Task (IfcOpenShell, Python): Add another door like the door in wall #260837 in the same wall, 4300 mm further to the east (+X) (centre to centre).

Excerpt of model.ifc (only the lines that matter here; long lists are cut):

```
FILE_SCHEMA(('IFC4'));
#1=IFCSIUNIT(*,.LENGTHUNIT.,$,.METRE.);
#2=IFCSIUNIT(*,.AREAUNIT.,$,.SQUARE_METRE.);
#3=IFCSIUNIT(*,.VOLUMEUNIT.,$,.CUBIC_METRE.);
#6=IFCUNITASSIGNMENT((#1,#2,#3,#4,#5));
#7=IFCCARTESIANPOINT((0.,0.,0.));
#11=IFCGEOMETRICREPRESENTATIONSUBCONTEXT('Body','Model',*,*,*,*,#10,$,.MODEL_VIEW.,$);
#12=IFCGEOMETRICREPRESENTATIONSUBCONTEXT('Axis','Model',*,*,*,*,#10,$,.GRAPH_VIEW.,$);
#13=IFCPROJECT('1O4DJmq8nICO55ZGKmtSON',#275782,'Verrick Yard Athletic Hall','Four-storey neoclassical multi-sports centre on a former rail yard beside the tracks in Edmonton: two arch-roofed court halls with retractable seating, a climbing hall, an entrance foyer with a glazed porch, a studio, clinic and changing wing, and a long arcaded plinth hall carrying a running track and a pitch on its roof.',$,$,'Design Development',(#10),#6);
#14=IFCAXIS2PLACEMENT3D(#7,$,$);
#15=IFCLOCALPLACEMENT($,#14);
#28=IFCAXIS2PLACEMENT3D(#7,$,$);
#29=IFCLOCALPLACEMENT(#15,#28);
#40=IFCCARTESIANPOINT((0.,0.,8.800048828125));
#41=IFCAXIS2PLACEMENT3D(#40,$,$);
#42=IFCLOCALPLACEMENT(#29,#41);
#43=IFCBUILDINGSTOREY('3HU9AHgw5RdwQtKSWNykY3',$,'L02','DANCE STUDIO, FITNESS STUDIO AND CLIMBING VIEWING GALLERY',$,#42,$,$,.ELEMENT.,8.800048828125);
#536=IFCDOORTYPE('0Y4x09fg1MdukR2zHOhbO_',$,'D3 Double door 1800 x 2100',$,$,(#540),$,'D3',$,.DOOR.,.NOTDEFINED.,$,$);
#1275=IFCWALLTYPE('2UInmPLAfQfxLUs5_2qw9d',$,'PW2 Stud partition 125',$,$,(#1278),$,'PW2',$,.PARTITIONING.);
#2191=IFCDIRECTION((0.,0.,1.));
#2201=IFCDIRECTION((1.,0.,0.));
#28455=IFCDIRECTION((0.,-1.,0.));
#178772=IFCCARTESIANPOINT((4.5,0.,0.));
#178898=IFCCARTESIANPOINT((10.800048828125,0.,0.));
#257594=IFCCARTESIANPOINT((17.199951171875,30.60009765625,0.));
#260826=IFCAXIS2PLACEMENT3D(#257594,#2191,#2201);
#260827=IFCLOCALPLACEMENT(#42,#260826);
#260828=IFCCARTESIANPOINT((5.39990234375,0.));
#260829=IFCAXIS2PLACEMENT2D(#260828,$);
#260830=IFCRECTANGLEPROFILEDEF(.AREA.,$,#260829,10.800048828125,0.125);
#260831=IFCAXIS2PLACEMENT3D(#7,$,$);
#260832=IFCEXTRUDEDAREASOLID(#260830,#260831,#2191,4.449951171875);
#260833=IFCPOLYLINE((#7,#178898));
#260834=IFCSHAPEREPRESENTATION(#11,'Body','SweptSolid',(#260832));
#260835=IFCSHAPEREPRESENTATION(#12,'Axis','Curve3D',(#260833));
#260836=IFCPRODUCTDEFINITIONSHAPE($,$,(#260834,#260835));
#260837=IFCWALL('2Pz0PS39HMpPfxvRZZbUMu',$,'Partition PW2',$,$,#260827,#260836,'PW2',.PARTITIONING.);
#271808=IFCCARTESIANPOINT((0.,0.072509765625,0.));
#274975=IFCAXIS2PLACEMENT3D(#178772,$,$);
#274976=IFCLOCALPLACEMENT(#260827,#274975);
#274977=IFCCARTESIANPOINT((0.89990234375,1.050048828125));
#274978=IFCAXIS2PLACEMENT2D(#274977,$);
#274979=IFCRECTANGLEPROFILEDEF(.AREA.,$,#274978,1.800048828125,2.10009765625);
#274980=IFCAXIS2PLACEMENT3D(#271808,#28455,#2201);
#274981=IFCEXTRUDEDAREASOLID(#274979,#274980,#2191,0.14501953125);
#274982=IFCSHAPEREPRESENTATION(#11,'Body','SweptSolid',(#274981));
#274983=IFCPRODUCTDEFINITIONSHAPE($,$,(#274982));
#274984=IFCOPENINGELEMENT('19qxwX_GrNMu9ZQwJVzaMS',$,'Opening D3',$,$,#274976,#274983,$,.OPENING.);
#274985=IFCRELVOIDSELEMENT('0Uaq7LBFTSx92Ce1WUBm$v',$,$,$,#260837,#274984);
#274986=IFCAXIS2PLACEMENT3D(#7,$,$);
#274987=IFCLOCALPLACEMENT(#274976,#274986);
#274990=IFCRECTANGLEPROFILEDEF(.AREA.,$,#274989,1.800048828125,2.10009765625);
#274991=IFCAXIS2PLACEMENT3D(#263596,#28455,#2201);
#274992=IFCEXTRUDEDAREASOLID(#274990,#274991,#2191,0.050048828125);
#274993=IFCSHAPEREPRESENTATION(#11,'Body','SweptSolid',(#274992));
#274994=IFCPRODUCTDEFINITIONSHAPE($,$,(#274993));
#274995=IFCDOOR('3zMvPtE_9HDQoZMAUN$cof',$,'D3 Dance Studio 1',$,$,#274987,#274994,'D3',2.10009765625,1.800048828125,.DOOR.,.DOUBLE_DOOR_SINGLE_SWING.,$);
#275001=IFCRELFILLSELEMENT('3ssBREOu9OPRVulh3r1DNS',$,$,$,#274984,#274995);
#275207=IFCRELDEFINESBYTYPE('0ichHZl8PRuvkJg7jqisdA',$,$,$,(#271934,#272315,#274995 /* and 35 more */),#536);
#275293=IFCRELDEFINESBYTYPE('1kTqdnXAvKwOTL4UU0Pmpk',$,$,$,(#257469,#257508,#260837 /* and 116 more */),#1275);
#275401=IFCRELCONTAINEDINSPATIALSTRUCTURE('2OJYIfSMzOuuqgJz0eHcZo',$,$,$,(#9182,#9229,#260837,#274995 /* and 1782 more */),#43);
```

```python
import ifcopenshell
import ifcopenshell.api.feature
import ifcopenshell.api.geometry
import ifcopenshell.api.root
import ifcopenshell.geom
import ifcopenshell.util.element
import ifcopenshell.util.placement
import ifcopenshell.util.shape

model = ifcopenshell.open("model.ifc")
settings = ifcopenshell.geom.settings()


def volume(element):
    """Net volume in cubic metres, openings subtracted."""
    shape = ifcopenshell.geom.create_shape(settings, element)
    return ifcopenshell.util.shape.get_volume(shape.geometry)


door = model.by_guid("3zMvPtE_9HDQoZMAUN$cof")
opening = door.FillsVoids[0].RelatingOpeningElement
wall = opening.VoidsElements[0].RelatingBuildingElement
before = volume(wall)
shift = ifcopenshell.util.placement.get_local_placement(wall.ObjectPlacement)[:3, 0] * 4.3

# copy_class copies the void relationship, type, container and properties, but no geometry.
new_opening = ifcopenshell.api.root.copy_class(model, product=opening)
new_opening.Representation = ifcopenshell.util.element.copy_deep(
    model, opening.Representation, exclude=["IfcGeometricRepresentationContext", "IfcRepresentationMap"]
)
new_door = ifcopenshell.api.root.copy_class(model, product=door)
new_door.Representation = ifcopenshell.util.element.copy_deep(
    model, door.Representation, exclude=["IfcGeometricRepresentationContext", "IfcRepresentationMap"]
)
new_door.Tag = None
ifcopenshell.api.feature.add_filling(model, opening=new_opening, element=new_door)

for old, new in ((opening, new_opening), (door, new_door)):
    matrix = ifcopenshell.util.placement.get_local_placement(old.ObjectPlacement)
    matrix[:3, 3] += shift
    ifcopenshell.api.geometry.edit_object_placement(model, product=new, matrix=matrix, is_si=False)

after = volume(wall)

print(f"wall volume {before:.3f} -> {after:.3f} m3")

model.write("model_updated.ifc")
```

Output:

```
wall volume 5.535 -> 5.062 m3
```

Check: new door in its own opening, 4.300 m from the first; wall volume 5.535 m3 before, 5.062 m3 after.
